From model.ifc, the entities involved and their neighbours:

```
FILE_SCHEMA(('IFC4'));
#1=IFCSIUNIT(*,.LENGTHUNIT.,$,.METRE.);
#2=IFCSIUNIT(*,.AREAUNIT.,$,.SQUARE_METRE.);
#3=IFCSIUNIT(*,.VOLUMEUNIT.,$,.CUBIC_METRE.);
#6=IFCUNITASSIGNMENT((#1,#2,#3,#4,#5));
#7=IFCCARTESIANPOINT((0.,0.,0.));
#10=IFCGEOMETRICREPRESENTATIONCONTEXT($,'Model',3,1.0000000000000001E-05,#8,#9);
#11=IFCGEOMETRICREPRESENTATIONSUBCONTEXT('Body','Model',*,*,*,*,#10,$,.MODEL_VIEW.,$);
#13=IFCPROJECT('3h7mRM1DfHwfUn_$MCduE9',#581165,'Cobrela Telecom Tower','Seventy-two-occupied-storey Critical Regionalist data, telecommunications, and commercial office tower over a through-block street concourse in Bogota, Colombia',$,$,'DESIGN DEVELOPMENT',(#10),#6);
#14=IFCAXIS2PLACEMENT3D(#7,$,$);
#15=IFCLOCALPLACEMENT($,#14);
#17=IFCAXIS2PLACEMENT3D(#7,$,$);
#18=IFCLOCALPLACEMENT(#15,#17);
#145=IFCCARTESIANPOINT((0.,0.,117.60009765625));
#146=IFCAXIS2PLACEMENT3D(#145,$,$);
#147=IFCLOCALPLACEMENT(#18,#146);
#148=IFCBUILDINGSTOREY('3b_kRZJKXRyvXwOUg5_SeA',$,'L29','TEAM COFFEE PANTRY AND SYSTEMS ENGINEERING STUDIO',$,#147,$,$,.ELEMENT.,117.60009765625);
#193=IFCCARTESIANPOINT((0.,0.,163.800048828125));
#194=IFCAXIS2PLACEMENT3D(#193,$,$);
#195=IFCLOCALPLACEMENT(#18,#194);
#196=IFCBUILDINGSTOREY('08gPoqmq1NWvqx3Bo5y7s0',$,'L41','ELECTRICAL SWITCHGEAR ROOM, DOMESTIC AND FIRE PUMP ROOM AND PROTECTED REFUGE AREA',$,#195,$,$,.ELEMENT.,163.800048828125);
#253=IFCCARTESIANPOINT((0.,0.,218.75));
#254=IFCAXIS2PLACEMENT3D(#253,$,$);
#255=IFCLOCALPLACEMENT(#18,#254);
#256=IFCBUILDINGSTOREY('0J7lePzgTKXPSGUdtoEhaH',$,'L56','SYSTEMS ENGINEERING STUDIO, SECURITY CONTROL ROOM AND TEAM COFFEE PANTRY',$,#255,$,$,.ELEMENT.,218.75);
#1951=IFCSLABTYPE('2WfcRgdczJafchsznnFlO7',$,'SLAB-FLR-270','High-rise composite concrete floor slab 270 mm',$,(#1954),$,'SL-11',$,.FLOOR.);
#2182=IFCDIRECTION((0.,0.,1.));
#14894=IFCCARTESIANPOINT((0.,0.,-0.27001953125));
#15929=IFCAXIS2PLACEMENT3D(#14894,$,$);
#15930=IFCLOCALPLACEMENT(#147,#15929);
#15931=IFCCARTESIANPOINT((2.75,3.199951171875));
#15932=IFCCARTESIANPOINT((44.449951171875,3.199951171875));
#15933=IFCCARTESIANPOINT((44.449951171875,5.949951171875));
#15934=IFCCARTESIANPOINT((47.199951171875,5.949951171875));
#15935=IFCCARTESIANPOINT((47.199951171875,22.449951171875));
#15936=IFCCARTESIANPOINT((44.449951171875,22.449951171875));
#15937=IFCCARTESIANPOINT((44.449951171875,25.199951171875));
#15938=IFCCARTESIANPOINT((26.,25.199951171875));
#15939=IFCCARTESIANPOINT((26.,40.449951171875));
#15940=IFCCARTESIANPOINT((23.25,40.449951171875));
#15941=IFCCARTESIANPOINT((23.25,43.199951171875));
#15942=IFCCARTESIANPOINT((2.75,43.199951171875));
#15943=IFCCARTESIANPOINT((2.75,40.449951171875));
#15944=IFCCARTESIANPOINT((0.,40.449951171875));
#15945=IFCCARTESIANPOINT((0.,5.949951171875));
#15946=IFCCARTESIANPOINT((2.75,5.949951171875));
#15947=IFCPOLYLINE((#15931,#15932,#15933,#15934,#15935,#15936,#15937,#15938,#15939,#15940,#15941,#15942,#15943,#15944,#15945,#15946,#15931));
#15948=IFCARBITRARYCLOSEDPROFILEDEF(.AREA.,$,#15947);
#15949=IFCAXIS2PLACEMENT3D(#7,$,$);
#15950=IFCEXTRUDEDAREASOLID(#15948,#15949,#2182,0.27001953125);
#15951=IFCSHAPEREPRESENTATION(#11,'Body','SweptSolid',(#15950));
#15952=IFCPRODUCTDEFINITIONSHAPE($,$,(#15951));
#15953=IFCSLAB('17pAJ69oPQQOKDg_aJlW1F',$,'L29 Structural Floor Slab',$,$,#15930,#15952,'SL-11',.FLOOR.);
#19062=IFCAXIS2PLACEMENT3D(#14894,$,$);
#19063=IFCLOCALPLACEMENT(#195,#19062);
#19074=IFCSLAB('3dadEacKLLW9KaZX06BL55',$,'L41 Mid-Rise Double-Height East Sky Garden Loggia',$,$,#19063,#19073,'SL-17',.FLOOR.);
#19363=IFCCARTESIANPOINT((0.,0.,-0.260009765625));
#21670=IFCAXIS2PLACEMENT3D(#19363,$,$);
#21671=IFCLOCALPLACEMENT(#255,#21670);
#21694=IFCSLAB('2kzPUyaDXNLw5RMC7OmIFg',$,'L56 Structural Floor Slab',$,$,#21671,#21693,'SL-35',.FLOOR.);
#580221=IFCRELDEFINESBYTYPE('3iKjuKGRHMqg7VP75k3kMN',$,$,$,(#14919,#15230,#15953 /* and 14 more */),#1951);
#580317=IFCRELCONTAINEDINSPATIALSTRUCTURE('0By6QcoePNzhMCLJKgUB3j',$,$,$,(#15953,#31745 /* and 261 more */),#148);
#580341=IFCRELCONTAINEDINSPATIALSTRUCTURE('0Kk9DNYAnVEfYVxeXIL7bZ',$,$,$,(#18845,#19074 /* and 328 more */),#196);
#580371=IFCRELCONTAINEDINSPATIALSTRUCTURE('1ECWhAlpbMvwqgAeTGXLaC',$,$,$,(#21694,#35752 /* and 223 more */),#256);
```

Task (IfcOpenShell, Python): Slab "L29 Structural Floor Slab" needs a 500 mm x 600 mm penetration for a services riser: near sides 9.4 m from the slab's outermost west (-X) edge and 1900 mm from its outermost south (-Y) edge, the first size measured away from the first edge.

```python
import numpy as np
import ifcopenshell
import ifcopenshell.api.feature
import ifcopenshell.api.geometry
import ifcopenshell.api.root
import ifcopenshell.geom
import ifcopenshell.util.placement
import ifcopenshell.util.representation
import ifcopenshell.util.shape
import ifcopenshell.util.unit

model = ifcopenshell.open("model.ifc")
unit_scale = ifcopenshell.util.unit.calculate_unit_scale(model)
settings = ifcopenshell.geom.settings()


def volume(element):
    """Net volume in cubic metres, openings subtracted."""
    shape = ifcopenshell.geom.create_shape(settings, element)
    return ifcopenshell.util.shape.get_volume(shape.geometry)


slab = model.by_guid("17pAJ69oPQQOKDg_aJlW1F")
before = volume(slab)

# Extent in the slab's own axes, in metres. The edges named are its -X and -Y sides.
slab_shape = ifcopenshell.geom.create_shape(settings, slab)
vertices = ifcopenshell.util.shape.get_vertices(slab_shape.geometry)
x_min, y_min, bottom = vertices.min(axis=0)
top = vertices[:, 2].max()

opening = ifcopenshell.api.root.create_entity(model, ifc_class="IfcOpeningElement", name="Services riser opening", predefined_type="OPENING")
context = ifcopenshell.util.representation.get_context(model, "Model", "Body", "MODEL_VIEW")
width, depth = 0.5, 0.6
outline = [(0.0, 0.0), (width, 0.0), (width, depth), (0.0, depth), (0.0, 0.0)]
# Overshoot both faces by 50 mm so the cut is clean.
shape = ifcopenshell.api.geometry.add_slab_representation(
    model, context=context, depth=top - bottom + 0.1, polyline=outline
)
ifcopenshell.api.geometry.assign_representation(model, product=opening, representation=shape)

matrix = ifcopenshell.util.placement.get_local_placement(slab.ObjectPlacement)
matrix[:, 3] = matrix @ np.append(np.array([x_min + 9.4, y_min + 1.9, bottom - 0.05]) / unit_scale, 1.0)
ifcopenshell.api.geometry.edit_object_placement(model, product=opening, matrix=matrix, is_si=False)
ifcopenshell.api.feature.add_feature(model, feature=opening, element=slab)

after = volume(slab)

print(f"slab volume {before:.3f} -> {after:.3f} m3")

model.write("model_rev.ifc")
```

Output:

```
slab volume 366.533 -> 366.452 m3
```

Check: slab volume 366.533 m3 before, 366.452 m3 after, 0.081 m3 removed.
